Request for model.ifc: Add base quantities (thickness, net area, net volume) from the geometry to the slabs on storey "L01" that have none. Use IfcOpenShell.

First a look at what the model holds.

```python
import ifcopenshell
import ifcopenshell.util.element
import ifcopenshell.util.unit

model = ifcopenshell.open("model.ifc")
print(model.schema)
for unit_type in ("LENGTHUNIT", "AREAUNIT", "VOLUMEUNIT"):
    print(unit_type, ifcopenshell.util.unit.calculate_unit_scale(model, unit_type))
storey = next(s for s in model.by_type("IfcBuildingStorey") if s.Name == "L01")
slabs = [e for e in ifcopenshell.util.element.get_decomposition(storey) if e.is_a("IfcSlab")]
for e in sorted(slabs, key=lambda e: e.id()):
    print(e.id(), e.is_a(), e.Name, list(ifcopenshell.util.element.get_psets(e, qtos_only=True)), sep=" | ")
```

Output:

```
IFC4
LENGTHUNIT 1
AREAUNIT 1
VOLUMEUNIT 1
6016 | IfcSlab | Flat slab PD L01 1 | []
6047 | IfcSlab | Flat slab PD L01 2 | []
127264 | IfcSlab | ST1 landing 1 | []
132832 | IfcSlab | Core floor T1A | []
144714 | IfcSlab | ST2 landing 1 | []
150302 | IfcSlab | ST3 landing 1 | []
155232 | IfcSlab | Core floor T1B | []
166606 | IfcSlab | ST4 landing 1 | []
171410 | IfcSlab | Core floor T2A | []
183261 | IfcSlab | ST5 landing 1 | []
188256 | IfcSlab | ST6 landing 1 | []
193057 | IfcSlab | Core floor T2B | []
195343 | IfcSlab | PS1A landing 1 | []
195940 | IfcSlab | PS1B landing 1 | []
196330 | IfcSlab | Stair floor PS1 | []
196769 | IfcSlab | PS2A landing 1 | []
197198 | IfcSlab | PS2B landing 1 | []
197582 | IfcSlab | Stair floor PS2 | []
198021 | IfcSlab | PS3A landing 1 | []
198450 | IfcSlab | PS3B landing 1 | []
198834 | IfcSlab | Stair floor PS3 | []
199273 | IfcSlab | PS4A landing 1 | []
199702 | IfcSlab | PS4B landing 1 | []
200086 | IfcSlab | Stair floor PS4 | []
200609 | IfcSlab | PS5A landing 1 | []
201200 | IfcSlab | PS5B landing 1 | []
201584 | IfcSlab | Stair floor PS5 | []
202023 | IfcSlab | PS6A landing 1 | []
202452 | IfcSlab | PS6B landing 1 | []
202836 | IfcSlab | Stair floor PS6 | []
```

```python
import ifcopenshell
import ifcopenshell.api.pset
import ifcopenshell.geom
import ifcopenshell.util.element
import ifcopenshell.util.shape
import ifcopenshell.util.unit

model = ifcopenshell.open("model.ifc")
unit_scale = ifcopenshell.util.unit.calculate_unit_scale(model)
area_scale = ifcopenshell.util.unit.calculate_unit_scale(model, "AREAUNIT")
volume_scale = ifcopenshell.util.unit.calculate_unit_scale(model, "VOLUMEUNIT")
settings = ifcopenshell.geom.settings()

storey = next(s for s in model.by_type("IfcBuildingStorey") if s.Name == "L01")
slabs = [e for e in ifcopenshell.util.element.get_decomposition(storey) if e.is_a("IfcSlab")]

for e in sorted(slabs, key=lambda e: e.id()):
    if ifcopenshell.util.element.get_psets(e, qtos_only=True, should_inherit=False):
        continue
    # Geometry comes back in metres, in the element's own axes.
    shape = ifcopenshell.geom.create_shape(settings, e)
    values = {
        "Width": ifcopenshell.util.shape.get_z(shape.geometry) / unit_scale,
        "NetArea": ifcopenshell.util.shape.get_footprint_area(shape.geometry) / area_scale,
        "NetVolume": ifcopenshell.util.shape.get_volume(shape.geometry) / volume_scale,
    }
    qto = ifcopenshell.api.pset.add_qto(model, product=e, name="Qto_SlabBaseQuantities")
    ifcopenshell.api.pset.edit_qto(model, qto=qto, properties=values)
    print(e.id(), {k: round(v, 3) for k, v in values.items()})

model.write("model_updated.ifc")
```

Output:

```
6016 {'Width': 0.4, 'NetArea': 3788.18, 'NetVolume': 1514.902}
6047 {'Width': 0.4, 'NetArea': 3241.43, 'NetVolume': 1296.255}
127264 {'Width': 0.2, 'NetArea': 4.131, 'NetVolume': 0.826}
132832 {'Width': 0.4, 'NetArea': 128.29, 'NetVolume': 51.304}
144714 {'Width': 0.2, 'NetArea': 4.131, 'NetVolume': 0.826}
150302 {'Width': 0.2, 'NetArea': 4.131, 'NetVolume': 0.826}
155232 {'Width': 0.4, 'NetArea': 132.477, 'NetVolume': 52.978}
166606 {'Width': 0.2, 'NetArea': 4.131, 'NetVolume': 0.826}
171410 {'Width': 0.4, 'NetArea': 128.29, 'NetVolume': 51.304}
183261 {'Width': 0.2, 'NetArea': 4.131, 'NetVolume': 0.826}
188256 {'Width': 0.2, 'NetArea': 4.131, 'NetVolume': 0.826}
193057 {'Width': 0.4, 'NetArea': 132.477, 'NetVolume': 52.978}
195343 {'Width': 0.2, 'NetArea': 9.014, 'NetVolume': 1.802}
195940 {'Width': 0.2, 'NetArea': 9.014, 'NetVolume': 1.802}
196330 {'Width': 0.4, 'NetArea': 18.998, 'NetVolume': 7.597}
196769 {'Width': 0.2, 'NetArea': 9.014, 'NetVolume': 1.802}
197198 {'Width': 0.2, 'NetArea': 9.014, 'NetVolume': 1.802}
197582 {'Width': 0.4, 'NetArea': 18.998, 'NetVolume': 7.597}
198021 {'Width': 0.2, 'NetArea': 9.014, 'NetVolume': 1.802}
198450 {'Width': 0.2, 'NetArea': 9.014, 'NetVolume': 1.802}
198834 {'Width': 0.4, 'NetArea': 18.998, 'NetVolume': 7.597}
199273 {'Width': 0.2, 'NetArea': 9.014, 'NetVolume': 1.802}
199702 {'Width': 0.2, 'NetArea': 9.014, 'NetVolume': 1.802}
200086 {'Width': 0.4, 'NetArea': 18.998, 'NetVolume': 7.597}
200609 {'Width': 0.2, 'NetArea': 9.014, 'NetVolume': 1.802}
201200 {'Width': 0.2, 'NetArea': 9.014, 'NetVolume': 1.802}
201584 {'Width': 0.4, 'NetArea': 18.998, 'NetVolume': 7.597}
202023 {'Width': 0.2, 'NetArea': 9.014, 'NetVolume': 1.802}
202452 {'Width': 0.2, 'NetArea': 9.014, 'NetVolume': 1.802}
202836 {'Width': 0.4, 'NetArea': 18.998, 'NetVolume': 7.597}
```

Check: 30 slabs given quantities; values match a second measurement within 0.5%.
